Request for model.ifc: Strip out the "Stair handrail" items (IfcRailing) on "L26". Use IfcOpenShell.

First a look at what the model holds.

```python
import ifcopenshell
import ifcopenshell.util.element

model = ifcopenshell.open("model.ifc")
print(model.schema)
storey = next(s for s in model.by_type("IfcBuildingStorey") if s.Name == "L26")
railings = [e for e in ifcopenshell.util.element.get_decomposition(storey) if e.is_a("IfcRailing")]
seen = {}
for e in railings:
    element_type = ifcopenshell.util.element.get_type(e)
    name = element_type.Name if element_type not in (None, e) else None
    seen[name] = seen.get(name, 0) + 1
for name, count in sorted(seen.items(), key=str):
    print(count, "x", name)
```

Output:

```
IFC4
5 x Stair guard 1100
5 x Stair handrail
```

```python
import ifcopenshell
import ifcopenshell.api.root
import ifcopenshell.util.element

model = ifcopenshell.open("model.ifc")

storey = next(s for s in model.by_type("IfcBuildingStorey") if s.Name == "L26")
railings = [e for e in ifcopenshell.util.element.get_decomposition(storey) if e.is_a("IfcRailing")]
targets = [e for e in railings if (t := ifcopenshell.util.element.get_type(e)) not in (None, e) and t.Name == "Stair handrail"]

for e in targets:
    ifcopenshell.api.root.remove_product(model, product=e)
print(len(targets), "removed")

model.write("model_updated.ifc")
```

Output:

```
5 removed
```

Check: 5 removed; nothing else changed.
